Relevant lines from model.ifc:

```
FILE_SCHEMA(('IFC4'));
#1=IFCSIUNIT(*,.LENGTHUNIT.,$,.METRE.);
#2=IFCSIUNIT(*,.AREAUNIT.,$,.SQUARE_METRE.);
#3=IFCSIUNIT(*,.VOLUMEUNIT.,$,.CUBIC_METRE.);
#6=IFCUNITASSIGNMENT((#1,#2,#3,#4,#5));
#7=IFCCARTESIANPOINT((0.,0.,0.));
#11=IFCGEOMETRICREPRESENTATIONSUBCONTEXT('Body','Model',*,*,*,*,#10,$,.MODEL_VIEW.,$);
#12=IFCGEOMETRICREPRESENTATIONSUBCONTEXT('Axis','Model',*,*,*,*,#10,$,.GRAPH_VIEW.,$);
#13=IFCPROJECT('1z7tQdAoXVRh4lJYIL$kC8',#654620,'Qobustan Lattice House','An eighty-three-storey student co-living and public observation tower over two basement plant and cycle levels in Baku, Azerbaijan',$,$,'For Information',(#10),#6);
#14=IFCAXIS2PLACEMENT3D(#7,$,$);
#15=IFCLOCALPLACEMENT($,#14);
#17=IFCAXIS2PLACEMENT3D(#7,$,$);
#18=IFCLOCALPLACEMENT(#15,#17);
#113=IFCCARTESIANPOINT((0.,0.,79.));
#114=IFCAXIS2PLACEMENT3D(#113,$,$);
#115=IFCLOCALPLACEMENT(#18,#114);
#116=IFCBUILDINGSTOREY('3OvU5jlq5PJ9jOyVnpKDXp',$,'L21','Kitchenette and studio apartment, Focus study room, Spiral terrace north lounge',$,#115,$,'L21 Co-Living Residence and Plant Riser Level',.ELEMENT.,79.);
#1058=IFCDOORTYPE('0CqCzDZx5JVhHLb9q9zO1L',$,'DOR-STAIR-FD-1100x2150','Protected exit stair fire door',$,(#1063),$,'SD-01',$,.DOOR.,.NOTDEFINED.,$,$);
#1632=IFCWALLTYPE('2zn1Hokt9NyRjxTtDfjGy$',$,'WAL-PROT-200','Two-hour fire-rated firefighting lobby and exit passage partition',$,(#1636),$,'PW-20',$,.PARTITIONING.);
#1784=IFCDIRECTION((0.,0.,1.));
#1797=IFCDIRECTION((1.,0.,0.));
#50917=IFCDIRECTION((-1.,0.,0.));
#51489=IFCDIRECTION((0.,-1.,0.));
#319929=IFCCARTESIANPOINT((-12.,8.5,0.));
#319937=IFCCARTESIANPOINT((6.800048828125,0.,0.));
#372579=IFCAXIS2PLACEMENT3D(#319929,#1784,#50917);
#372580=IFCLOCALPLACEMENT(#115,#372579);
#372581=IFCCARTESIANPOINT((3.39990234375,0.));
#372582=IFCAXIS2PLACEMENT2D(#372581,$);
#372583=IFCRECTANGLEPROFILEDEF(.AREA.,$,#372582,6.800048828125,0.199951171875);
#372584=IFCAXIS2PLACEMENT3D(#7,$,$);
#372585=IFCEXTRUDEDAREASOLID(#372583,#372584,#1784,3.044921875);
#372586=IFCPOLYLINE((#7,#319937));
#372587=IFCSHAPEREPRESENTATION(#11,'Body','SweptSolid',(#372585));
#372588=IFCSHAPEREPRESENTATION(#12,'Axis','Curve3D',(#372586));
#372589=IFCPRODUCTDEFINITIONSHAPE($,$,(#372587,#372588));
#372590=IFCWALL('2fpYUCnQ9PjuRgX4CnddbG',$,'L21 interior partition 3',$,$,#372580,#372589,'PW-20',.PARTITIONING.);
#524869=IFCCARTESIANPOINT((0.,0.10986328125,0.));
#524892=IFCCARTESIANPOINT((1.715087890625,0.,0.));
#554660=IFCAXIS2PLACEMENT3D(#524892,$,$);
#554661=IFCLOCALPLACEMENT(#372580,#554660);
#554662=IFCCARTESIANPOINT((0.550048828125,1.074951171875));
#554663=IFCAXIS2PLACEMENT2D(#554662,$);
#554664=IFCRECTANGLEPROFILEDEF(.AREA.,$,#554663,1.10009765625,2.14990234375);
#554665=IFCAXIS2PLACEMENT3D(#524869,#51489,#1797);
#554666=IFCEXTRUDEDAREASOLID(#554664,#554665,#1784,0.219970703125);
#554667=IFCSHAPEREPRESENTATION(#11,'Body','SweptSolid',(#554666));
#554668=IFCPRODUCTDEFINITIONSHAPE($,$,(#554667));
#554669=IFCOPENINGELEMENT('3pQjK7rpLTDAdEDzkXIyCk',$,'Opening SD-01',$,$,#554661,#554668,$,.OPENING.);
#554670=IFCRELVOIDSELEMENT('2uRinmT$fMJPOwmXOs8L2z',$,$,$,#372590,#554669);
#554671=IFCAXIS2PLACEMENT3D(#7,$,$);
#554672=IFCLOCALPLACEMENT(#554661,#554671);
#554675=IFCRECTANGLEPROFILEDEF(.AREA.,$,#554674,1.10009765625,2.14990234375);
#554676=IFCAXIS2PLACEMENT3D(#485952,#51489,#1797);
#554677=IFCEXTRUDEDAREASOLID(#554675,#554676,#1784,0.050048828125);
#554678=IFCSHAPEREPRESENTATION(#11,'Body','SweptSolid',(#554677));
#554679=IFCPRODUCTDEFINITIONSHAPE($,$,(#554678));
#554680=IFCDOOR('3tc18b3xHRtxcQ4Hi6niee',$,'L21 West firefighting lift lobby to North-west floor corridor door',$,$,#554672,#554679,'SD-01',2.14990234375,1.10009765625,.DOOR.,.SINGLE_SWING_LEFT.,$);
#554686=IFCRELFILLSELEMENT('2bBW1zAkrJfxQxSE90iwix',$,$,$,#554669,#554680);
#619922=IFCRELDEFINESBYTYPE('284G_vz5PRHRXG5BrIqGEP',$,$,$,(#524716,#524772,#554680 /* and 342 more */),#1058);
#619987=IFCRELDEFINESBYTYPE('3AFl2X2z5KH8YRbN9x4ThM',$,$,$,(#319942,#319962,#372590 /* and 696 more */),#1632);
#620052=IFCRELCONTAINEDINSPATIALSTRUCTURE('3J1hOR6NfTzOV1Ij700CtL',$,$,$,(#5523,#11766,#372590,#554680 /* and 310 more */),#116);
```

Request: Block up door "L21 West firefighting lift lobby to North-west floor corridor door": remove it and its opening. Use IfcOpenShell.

```python
import ifcopenshell
import ifcopenshell.api.feature
import ifcopenshell.api.root
import ifcopenshell.geom
import ifcopenshell.util.shape

model = ifcopenshell.open("model.ifc")
settings = ifcopenshell.geom.settings()


def volume(element):
    """Net volume in cubic metres, openings subtracted."""
    shape = ifcopenshell.geom.create_shape(settings, element)
    return ifcopenshell.util.shape.get_volume(shape.geometry)


door = model.by_guid("3tc18b3xHRtxcQ4Hi6niee")
opening = door.FillsVoids[0].RelatingOpeningElement
wall = opening.VoidsElements[0].RelatingBuildingElement
before = volume(wall)

ifcopenshell.api.root.remove_product(model, product=door)
ifcopenshell.api.feature.remove_feature(model, feature=opening)

after = volume(wall)

print(f"wall volume {before:.3f} -> {after:.3f} m3")

model.write("model_v2.ifc")
```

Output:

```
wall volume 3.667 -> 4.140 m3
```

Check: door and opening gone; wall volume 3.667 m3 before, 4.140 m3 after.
